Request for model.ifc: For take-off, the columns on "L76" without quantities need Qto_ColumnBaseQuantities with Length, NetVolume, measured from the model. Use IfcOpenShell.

First a look at what the model holds.

```python
import ifcopenshell
import ifcopenshell.util.element
import ifcopenshell.util.unit

model = ifcopenshell.open("model.ifc")
print(model.schema)
for unit_type in ("LENGTHUNIT", "AREAUNIT", "VOLUMEUNIT"):
    print(unit_type, ifcopenshell.util.unit.calculate_unit_scale(model, unit_type))
storey = next(s for s in model.by_type("IfcBuildingStorey") if s.Name == "L76")
columns = [e for e in ifcopenshell.util.element.get_decomposition(storey) if e.is_a("IfcColumn")]
for e in sorted(columns, key=lambda e: e.id()):
    print(e.id(), e.is_a(), e.Name, list(ifcopenshell.util.element.get_psets(e, qtos_only=True)), sep=" | ")
```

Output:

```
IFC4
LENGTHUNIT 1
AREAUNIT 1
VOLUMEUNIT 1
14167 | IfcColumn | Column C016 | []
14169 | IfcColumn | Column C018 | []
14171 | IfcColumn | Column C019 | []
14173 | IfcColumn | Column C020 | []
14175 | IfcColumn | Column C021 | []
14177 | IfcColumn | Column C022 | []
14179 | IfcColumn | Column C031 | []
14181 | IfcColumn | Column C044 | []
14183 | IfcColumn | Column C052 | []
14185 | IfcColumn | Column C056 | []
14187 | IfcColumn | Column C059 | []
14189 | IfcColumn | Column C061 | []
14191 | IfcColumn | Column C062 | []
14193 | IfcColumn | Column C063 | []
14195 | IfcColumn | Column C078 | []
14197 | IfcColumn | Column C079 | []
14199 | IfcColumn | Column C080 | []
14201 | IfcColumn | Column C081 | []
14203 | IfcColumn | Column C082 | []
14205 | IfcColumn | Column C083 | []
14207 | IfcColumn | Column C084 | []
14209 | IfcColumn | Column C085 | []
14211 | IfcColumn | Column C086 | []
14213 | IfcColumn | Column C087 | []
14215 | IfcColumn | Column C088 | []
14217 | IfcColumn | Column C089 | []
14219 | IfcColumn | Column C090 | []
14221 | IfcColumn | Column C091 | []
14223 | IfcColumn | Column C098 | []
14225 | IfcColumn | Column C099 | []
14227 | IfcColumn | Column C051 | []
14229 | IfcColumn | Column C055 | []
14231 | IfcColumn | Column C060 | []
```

```python
import ifcopenshell
import ifcopenshell.api.pset
import ifcopenshell.geom
import ifcopenshell.util.element
import ifcopenshell.util.shape
import ifcopenshell.util.unit

model = ifcopenshell.open("model.ifc")
unit_scale = ifcopenshell.util.unit.calculate_unit_scale(model)
volume_scale = ifcopenshell.util.unit.calculate_unit_scale(model, "VOLUMEUNIT")
settings = ifcopenshell.geom.settings()

storey = next(s for s in model.by_type("IfcBuildingStorey") if s.Name == "L76")
columns = [e for e in ifcopenshell.util.element.get_decomposition(storey) if e.is_a("IfcColumn")]

for e in sorted(columns, key=lambda e: e.id()):
    if ifcopenshell.util.element.get_psets(e, qtos_only=True, should_inherit=False):
        continue
    # Geometry comes back in metres, in the element's own axes.
    shape = ifcopenshell.geom.create_shape(settings, e)
    values = {
        "Length": ifcopenshell.util.shape.get_z(shape.geometry) / unit_scale,
        "NetVolume": ifcopenshell.util.shape.get_volume(shape.geometry) / volume_scale,
    }
    qto = ifcopenshell.api.pset.add_qto(model, product=e, name="Qto_ColumnBaseQuantities")
    ifcopenshell.api.pset.edit_qto(model, qto=qto, properties=values)
    print(e.id(), {k: round(v, 3) for k, v in values.items()})

model.write("model_v2.ifc")
```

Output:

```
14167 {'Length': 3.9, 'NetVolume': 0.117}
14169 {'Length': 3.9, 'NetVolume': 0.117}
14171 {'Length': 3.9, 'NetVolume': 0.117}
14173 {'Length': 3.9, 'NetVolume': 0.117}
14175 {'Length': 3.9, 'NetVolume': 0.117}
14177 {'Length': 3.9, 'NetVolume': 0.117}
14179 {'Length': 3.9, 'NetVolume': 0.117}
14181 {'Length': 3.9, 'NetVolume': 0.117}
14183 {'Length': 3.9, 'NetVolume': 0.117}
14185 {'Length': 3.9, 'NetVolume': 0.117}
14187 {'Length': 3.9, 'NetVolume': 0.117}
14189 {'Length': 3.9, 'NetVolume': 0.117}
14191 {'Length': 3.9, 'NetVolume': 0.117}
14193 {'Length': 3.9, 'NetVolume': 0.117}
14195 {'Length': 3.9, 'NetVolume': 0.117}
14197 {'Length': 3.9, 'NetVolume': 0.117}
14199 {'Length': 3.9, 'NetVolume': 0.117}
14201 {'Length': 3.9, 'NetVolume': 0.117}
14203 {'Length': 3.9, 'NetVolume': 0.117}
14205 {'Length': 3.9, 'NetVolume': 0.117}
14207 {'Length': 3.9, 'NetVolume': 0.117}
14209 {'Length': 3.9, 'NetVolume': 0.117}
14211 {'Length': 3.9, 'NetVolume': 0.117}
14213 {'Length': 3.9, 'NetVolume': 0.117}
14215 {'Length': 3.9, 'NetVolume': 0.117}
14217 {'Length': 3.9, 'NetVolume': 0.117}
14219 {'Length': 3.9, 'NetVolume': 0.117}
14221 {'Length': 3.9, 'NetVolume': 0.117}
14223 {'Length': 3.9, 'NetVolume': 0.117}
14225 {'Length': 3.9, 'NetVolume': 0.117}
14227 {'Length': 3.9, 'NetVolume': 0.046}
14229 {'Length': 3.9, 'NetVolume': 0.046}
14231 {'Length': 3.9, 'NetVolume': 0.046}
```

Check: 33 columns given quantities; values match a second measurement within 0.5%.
